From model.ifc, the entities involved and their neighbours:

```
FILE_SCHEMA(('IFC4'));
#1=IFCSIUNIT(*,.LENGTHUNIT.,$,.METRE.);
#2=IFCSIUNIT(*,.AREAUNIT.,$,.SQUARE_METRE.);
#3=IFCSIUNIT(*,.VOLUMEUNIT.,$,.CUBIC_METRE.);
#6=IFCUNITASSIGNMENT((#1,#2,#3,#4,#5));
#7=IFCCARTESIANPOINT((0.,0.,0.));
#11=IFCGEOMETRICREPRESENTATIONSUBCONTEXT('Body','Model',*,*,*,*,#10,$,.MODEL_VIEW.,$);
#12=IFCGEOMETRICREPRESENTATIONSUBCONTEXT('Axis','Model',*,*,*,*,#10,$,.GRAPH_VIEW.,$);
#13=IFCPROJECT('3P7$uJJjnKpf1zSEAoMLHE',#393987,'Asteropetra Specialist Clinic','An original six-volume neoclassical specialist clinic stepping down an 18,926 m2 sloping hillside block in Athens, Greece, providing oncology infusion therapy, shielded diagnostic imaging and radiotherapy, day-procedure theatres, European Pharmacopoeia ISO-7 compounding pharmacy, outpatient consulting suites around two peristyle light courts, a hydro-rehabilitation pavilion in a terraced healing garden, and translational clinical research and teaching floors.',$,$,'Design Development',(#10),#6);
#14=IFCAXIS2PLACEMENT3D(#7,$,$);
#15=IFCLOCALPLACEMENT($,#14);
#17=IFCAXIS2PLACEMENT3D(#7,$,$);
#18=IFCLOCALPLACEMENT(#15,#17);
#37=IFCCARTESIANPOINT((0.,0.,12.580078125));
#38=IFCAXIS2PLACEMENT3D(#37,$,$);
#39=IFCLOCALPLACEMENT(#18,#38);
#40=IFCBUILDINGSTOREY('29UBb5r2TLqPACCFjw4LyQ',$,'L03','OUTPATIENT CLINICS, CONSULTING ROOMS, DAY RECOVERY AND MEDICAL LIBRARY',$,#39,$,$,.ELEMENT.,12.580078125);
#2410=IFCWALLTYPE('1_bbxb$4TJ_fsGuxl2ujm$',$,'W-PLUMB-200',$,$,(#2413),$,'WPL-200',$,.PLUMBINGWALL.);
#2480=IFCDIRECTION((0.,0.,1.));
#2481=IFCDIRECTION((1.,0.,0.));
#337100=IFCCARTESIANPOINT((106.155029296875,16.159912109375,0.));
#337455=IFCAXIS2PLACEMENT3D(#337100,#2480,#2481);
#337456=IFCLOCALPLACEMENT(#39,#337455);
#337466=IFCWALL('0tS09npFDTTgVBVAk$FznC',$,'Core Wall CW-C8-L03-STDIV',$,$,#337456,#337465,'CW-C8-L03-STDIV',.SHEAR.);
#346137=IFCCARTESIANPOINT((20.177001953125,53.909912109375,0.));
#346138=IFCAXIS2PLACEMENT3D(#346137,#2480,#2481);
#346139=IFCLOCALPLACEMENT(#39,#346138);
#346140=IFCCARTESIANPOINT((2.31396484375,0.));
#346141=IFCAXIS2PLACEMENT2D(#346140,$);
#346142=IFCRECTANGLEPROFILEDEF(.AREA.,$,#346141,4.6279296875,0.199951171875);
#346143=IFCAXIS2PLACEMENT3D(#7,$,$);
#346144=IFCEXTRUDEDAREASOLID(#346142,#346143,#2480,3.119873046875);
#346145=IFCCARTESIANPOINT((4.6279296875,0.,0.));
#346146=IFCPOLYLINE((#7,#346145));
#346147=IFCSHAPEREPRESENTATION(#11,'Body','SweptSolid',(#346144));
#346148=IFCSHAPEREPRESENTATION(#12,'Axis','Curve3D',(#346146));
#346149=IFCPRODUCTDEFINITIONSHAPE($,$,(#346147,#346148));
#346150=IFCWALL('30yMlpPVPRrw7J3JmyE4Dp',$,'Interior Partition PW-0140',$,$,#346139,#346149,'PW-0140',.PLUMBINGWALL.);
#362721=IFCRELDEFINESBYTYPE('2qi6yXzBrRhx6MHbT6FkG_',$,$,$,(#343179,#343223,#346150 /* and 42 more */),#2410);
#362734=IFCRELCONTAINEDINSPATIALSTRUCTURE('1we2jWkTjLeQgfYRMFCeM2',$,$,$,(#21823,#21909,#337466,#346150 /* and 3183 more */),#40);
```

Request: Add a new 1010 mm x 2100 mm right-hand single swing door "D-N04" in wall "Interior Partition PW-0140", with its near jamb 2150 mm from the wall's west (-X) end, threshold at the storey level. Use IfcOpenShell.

```python
import numpy as np
import ifcopenshell
import ifcopenshell.api.feature
import ifcopenshell.api.geometry
import ifcopenshell.api.root
import ifcopenshell.api.spatial
import ifcopenshell.geom
import ifcopenshell.util.element
import ifcopenshell.util.placement
import ifcopenshell.util.representation
import ifcopenshell.util.shape
import ifcopenshell.util.unit

model = ifcopenshell.open("model.ifc")
unit_scale = ifcopenshell.util.unit.calculate_unit_scale(model)
settings = ifcopenshell.geom.settings()


def volume(element):
    """Net volume in cubic metres, openings subtracted."""
    shape = ifcopenshell.geom.create_shape(settings, element)
    return ifcopenshell.util.shape.get_volume(shape.geometry)


wall = model.by_guid("30yMlpPVPRrw7J3JmyE4Dp")
storey = ifcopenshell.util.element.get_container(wall, ifc_class="IfcBuildingStorey")
context = ifcopenshell.util.representation.get_context(model, "Model", "Body", "MODEL_VIEW")
before = volume(wall)

width, height, from_end, sill = 1.01, 2.1, 2.15, 0.0  # metres

# The wall runs along its own X axis, and the end named is its -X end.
wall_shape = ifcopenshell.geom.create_shape(settings, wall)
x, y, z = ifcopenshell.util.shape.get_vertices(wall_shape.geometry).T
start = x.min() + from_end
face, thickness = float(y.min()), float(y.max() - y.min())
wall_matrix = ifcopenshell.util.placement.get_local_placement(wall.ObjectPlacement)
level = ifcopenshell.util.placement.get_local_placement(storey.ObjectPlacement)[2, 3]


def in_wall(x, y):
    """Placement at x, y metres in the wall's axes, at sill height."""
    matrix = wall_matrix.copy()
    matrix[:, 3] = wall_matrix @ np.array([x / unit_scale, y / unit_scale, 0.0, 1.0])
    matrix[2, 3] = level + sill / unit_scale
    return matrix


# Opening: a box that overshoots both wall faces by 50 mm.
opening = ifcopenshell.api.root.create_entity(model, ifc_class="IfcOpeningElement", predefined_type="OPENING")
box = ifcopenshell.api.geometry.add_wall_representation(
    model, context=context, length=width, height=height, thickness=thickness + 0.1
)
ifcopenshell.api.geometry.assign_representation(model, product=opening, representation=box)
ifcopenshell.api.geometry.edit_object_placement(model, product=opening, matrix=in_wall(start, face - 0.05), is_si=False)
ifcopenshell.api.feature.add_feature(model, feature=opening, element=wall)

door = ifcopenshell.api.root.create_entity(model, ifc_class="IfcDoor", name="D-N04", predefined_type="DOOR")
door.OverallWidth, door.OverallHeight = width / unit_scale, height / unit_scale
door.OperationType = "SINGLE_SWING_RIGHT"
body = ifcopenshell.api.geometry.add_door_representation(
    model,
    context=context,
    overall_width=door.OverallWidth,
    overall_height=door.OverallHeight,
    operation_type="SINGLE_SWING_RIGHT",
    lining_properties={"LiningDepth": thickness / unit_scale, "ThresholdDepth": thickness / unit_scale},
)
ifcopenshell.api.geometry.assign_representation(model, product=door, representation=body)
ifcopenshell.api.spatial.assign_container(model, products=[door], relating_structure=storey)
ifcopenshell.api.feature.add_filling(model, opening=opening, element=door)

# The lining spans the wall, so the door starts at the wall face.
ifcopenshell.api.geometry.edit_object_placement(model, product=door, matrix=in_wall(start, face), is_si=False)

after = volume(wall)

print(f"wall volume {before:.3f} -> {after:.3f} m3")

model.write("model_v2.ifc")
```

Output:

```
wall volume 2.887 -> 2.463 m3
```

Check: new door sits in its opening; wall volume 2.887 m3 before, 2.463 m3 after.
